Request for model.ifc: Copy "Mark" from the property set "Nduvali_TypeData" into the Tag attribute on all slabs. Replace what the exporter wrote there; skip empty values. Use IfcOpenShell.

First a look at what the model holds.

```python
import ifcopenshell
import ifcopenshell.util.element

model = ifcopenshell.open("model.ifc")
print(model.schema)
slabs = model.by_type("IfcSlab")
print(len(slabs), "slabs")
for e in slabs[:8]:
    source = ifcopenshell.util.element.get_pset(e, "Nduvali_TypeData", "Mark")
    target = e.Tag
    print(e.id(), repr(source), repr(target), sep=" | ")
```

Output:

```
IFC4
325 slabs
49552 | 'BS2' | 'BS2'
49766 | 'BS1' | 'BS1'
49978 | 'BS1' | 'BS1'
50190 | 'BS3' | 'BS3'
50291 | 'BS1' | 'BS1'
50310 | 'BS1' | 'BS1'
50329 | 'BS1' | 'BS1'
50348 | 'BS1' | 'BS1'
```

```python
import ifcopenshell
import ifcopenshell.util.element

model = ifcopenshell.open("model.ifc")

count = 0
for e in model.by_type("IfcSlab"):
    value = ifcopenshell.util.element.get_pset(e, "Nduvali_TypeData", "Mark")
    current = e.Tag
    if not value or not value.strip() or current == value:
        continue
    e.Tag = value
    count += 1

print(count, "slabs updated")

model.write("model-out.ifc")
```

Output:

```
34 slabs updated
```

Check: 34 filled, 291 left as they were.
